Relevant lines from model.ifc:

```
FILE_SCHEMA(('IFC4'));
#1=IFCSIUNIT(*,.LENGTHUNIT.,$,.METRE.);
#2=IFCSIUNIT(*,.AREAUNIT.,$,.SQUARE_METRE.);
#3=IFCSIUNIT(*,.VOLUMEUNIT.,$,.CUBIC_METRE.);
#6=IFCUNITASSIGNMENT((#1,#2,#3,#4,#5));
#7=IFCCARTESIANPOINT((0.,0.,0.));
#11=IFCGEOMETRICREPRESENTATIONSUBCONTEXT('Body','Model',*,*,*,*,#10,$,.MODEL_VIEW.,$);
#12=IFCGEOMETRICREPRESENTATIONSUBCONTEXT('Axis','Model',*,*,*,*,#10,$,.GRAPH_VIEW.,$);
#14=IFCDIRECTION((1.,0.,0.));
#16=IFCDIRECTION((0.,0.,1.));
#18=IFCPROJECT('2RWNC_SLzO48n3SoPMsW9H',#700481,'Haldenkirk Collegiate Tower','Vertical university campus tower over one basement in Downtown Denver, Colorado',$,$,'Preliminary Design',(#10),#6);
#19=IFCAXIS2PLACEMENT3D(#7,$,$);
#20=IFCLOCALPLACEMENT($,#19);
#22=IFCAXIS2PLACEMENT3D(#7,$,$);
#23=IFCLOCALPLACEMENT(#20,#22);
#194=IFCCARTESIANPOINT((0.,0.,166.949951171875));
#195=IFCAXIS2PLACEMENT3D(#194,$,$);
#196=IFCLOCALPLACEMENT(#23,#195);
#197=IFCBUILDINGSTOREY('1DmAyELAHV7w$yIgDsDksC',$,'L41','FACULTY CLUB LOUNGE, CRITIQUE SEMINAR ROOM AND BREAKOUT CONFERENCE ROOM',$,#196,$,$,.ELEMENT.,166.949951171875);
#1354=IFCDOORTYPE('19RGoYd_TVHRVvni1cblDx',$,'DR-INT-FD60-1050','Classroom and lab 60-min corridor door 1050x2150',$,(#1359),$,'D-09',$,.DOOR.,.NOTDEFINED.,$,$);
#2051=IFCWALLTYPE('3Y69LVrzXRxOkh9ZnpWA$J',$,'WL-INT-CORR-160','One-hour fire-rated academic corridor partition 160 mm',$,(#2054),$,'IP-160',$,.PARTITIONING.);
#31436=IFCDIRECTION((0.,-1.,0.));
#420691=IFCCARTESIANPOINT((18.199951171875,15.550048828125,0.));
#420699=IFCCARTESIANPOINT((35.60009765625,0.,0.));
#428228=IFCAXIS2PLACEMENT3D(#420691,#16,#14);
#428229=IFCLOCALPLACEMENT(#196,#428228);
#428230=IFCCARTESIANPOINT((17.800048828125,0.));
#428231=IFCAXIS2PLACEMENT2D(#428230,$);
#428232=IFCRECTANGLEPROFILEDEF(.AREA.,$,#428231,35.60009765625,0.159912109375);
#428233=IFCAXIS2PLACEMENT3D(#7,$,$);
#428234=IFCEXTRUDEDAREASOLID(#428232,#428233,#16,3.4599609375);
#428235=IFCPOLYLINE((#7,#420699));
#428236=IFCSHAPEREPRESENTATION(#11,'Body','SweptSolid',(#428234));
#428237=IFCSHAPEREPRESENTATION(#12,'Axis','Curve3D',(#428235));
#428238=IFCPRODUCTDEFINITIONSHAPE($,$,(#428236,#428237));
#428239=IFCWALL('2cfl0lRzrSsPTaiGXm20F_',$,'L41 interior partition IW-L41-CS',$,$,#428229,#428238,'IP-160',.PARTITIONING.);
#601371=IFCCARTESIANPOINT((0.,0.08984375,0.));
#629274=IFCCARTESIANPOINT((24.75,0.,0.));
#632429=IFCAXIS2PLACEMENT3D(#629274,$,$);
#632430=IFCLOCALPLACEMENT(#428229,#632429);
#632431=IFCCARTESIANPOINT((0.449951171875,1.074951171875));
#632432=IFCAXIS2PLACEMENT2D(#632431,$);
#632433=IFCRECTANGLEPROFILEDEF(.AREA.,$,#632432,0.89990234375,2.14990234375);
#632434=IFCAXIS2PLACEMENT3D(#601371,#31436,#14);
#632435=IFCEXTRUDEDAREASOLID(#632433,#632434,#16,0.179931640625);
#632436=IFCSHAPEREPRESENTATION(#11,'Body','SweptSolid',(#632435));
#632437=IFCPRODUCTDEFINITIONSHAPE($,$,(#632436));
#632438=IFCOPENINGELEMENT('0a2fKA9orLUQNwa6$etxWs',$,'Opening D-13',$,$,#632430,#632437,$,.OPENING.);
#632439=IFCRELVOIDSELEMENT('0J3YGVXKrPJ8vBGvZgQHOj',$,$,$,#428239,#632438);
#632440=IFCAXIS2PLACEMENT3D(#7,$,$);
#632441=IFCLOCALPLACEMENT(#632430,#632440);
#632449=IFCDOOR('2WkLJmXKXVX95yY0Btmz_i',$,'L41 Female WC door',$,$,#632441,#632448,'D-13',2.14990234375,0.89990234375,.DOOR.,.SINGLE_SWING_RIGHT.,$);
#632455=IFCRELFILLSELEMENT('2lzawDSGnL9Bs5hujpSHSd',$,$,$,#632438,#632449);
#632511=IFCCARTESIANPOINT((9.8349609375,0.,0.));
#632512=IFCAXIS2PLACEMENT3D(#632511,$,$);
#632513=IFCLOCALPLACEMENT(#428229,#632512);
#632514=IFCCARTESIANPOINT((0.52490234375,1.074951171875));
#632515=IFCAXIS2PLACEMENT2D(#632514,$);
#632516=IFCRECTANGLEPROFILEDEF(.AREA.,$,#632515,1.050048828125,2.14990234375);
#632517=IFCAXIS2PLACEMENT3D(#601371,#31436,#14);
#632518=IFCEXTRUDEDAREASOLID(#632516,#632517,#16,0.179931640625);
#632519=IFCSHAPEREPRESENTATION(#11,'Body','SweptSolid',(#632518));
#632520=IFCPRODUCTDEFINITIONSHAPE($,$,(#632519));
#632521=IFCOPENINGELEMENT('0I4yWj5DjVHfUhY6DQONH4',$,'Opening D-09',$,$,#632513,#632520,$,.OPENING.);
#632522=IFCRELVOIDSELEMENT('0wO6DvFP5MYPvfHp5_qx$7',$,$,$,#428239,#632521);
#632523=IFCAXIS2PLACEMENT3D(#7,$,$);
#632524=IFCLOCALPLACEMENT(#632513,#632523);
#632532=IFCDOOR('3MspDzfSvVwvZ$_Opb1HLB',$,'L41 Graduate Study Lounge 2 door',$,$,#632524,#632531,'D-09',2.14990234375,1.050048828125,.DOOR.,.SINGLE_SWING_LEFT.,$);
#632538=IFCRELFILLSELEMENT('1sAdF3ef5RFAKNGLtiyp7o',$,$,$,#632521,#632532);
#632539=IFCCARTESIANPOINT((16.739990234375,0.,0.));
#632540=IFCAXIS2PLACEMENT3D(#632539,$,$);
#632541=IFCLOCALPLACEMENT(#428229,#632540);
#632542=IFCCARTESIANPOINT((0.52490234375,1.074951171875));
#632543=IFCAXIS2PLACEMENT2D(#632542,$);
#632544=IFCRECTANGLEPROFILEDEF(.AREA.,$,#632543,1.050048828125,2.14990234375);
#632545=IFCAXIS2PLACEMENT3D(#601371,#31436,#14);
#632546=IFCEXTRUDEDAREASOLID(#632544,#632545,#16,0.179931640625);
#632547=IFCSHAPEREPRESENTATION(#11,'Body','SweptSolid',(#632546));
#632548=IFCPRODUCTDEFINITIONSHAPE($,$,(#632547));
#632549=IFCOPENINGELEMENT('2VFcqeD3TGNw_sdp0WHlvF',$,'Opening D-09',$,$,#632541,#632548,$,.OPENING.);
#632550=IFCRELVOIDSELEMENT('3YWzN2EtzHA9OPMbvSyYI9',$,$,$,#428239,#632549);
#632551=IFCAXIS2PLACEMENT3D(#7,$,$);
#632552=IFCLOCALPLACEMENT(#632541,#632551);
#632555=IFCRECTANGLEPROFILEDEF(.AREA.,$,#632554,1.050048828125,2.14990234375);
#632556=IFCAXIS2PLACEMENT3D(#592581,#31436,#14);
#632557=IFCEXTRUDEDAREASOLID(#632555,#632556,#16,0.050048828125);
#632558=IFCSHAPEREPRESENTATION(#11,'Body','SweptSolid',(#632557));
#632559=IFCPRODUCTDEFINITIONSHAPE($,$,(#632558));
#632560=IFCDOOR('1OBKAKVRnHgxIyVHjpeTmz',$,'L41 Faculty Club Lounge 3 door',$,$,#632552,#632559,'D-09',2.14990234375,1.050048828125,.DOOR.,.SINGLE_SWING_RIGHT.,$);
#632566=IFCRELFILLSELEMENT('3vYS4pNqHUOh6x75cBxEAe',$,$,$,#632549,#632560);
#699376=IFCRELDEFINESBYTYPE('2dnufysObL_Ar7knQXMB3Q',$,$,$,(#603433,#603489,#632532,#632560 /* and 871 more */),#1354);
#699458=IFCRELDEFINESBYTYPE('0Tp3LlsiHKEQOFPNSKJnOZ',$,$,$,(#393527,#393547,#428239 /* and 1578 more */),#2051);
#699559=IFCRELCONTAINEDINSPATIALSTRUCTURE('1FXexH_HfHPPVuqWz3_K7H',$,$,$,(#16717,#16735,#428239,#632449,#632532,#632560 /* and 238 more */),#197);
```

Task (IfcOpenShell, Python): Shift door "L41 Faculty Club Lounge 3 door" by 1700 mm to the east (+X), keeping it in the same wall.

```python
import ifcopenshell
import ifcopenshell.api.geometry
import ifcopenshell.util.placement
import ifcopenshell.util.unit

model = ifcopenshell.open("model.ifc")
unit_scale = ifcopenshell.util.unit.calculate_unit_scale(model)

door = model.by_guid("1OBKAKVRnHgxIyVHjpeTmz")
opening = door.FillsVoids[0].RelatingOpeningElement
wall = opening.VoidsElements[0].RelatingBuildingElement

wall_matrix = ifcopenshell.util.placement.get_local_placement(wall.ObjectPlacement)
shift = wall_matrix[:3, 0] * 1.7 / unit_scale
before = ifcopenshell.util.placement.get_local_placement(door.ObjectPlacement)[:3, 3].copy()

# The door is placed relative to its opening, so it follows when the opening moves.
matrix = ifcopenshell.util.placement.get_local_placement(opening.ObjectPlacement)
matrix[:3, 3] += shift
ifcopenshell.api.geometry.edit_object_placement(
    model, product=opening, matrix=matrix, is_si=False, should_transform_children=True
)

after = ifcopenshell.util.placement.get_local_placement(door.ObjectPlacement)[:3, 3]
print("door moved by", (after - before).round(3) + 0.0)

model.write("model_rev.ifc")
```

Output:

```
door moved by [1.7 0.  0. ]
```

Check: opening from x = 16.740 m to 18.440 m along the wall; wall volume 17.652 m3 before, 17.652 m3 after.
